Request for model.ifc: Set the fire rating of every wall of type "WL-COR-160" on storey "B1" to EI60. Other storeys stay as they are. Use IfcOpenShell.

First a look at what the model holds.

```python
import ifcopenshell
import ifcopenshell.util.element

model = ifcopenshell.open("model.ifc")
print(model.schema)
storey = next(s for s in model.by_type("IfcBuildingStorey") if s.Name == "B1")
walls = [e for e in ifcopenshell.util.element.get_decomposition(storey) if e.is_a("IfcWall")]
seen = {}
for e in walls:
    element_type = ifcopenshell.util.element.get_type(e)
    key = (element_type.Name if element_type != e and element_type else None, ifcopenshell.util.element.get_pset(e, "Pset_WallCommon", "FireRating"))
    seen[key] = seen.get(key, 0) + 1
for (name, value), count in sorted(seen.items(), key=str):
    print(count, "x", name, "|", value)
```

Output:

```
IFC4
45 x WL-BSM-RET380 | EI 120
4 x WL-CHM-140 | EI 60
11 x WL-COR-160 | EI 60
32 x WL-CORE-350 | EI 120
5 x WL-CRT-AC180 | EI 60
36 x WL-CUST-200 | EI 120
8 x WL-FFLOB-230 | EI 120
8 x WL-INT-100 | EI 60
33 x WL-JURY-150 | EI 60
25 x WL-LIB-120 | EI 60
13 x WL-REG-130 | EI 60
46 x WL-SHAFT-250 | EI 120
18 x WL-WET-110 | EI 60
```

```python
import ifcopenshell
import ifcopenshell.api.pset
import ifcopenshell.util.element

model = ifcopenshell.open("model.ifc")

storey = next(s for s in model.by_type("IfcBuildingStorey") if s.Name == "B1")
walls = [e for e in ifcopenshell.util.element.get_decomposition(storey) if e.is_a("IfcWall")]

count = 0
for e in walls:
    element_type = ifcopenshell.util.element.get_type(e)
    if element_type in (None, e) or element_type.Name != "WL-COR-160":
        continue
    # add_pset returns the element's existing set when there is one.
    pset = ifcopenshell.api.pset.add_pset(model, product=e, name="Pset_WallCommon")
    ifcopenshell.api.pset.edit_pset(model, pset=pset, properties={"FireRating": "EI60"})
    count += 1

print(count, "walls updated")

model.write("model_rev.ifc")
```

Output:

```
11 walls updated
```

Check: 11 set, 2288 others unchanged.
